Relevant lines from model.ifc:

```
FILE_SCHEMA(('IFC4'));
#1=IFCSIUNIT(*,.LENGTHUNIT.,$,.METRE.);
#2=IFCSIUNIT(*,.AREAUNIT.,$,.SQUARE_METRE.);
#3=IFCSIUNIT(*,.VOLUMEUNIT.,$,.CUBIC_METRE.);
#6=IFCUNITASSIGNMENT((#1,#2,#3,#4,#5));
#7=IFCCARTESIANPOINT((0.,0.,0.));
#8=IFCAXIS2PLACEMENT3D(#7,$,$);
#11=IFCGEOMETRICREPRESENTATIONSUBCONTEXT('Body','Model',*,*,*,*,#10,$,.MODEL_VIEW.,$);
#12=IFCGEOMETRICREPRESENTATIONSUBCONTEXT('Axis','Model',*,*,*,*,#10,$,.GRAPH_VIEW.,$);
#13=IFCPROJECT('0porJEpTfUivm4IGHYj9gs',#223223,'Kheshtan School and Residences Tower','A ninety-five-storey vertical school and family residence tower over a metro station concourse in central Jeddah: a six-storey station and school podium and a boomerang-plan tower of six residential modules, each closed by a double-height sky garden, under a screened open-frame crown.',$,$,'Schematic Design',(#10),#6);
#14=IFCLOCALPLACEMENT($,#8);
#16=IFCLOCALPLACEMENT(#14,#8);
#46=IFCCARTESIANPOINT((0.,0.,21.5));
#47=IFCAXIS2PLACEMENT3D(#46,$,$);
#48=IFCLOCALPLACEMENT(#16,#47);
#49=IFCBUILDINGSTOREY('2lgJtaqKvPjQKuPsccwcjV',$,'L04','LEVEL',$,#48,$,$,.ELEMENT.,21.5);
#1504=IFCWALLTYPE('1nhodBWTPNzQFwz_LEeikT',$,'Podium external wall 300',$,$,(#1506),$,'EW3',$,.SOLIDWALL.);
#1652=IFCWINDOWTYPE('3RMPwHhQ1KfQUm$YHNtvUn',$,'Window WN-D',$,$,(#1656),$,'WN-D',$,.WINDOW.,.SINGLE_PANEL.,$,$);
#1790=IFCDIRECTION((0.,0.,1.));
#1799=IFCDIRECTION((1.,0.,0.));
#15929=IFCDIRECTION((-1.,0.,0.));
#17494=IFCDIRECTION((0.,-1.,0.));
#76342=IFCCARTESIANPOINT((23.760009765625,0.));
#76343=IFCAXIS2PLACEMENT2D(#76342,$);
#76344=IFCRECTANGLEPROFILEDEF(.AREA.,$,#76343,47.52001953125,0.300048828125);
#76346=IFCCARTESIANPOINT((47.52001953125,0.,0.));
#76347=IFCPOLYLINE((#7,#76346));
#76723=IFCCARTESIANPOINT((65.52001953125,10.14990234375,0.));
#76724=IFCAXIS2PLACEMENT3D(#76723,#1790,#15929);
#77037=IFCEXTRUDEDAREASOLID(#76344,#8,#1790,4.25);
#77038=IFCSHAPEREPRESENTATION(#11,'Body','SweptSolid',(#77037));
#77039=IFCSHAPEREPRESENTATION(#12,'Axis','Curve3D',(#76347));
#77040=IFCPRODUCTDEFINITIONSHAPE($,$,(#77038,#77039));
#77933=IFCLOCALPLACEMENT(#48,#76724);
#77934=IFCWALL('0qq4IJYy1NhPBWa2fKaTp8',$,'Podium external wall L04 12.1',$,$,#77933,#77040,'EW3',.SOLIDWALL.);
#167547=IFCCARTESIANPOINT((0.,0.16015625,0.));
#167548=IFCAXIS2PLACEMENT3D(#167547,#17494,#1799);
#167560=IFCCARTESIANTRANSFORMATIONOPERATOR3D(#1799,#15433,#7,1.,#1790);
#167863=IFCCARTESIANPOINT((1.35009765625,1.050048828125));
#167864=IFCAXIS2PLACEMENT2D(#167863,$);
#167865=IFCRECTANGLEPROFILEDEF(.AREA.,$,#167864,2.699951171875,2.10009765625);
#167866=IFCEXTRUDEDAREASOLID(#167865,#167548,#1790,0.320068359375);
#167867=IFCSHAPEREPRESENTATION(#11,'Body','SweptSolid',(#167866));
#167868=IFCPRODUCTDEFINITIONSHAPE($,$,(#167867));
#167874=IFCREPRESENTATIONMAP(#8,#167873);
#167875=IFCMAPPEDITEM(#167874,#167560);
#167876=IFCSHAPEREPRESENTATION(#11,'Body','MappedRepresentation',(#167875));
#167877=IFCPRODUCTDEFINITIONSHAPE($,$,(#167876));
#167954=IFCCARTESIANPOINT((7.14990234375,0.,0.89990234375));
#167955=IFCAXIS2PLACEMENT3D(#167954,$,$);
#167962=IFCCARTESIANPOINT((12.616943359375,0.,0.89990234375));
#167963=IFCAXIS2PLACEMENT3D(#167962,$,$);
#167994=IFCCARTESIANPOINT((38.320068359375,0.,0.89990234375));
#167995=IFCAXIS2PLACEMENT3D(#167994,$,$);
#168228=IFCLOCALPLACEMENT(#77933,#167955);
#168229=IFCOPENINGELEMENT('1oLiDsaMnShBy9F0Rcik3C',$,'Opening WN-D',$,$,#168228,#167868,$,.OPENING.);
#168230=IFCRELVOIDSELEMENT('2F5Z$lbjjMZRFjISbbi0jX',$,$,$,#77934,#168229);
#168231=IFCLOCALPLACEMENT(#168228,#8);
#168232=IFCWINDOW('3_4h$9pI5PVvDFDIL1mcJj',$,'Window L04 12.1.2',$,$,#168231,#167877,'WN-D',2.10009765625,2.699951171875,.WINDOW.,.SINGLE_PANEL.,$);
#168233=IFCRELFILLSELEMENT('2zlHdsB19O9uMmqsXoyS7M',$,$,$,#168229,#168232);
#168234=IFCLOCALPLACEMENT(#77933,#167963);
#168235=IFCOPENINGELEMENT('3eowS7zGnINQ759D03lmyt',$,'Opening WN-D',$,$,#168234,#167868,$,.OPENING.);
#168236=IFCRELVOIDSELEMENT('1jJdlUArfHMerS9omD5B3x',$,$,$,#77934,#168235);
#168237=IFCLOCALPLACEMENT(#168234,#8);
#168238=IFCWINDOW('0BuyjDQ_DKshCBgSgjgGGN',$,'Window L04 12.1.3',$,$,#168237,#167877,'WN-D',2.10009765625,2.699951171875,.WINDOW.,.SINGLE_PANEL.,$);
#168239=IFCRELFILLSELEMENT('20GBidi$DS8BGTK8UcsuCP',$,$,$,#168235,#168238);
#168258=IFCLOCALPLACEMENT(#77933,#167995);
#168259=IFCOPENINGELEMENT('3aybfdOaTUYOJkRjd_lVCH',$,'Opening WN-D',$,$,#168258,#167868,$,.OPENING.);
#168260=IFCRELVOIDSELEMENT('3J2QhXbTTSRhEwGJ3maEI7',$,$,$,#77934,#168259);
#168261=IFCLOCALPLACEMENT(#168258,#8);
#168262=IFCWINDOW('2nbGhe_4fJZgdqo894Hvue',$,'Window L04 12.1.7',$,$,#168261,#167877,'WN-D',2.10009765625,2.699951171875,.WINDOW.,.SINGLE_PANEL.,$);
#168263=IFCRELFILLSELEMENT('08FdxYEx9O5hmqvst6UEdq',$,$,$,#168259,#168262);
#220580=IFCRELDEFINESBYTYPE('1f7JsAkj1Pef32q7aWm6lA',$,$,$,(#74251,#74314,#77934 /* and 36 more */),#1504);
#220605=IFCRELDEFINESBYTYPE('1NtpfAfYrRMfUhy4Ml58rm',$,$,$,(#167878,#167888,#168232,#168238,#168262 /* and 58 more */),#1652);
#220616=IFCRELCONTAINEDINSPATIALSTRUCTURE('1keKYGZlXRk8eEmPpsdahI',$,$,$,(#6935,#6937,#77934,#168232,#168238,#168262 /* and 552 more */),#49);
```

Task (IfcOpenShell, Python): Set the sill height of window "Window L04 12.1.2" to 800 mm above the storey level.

```python
import numpy as np
import ifcopenshell
import ifcopenshell.api.geometry
import ifcopenshell.geom
import ifcopenshell.util.element
import ifcopenshell.util.placement
import ifcopenshell.util.shape
import ifcopenshell.util.unit

model = ifcopenshell.open("model.ifc")
unit_scale = ifcopenshell.util.unit.calculate_unit_scale(model)

window = model.by_guid("3_4h$9pI5PVvDFDIL1mcJj")
opening = window.FillsVoids[0].RelatingOpeningElement
storey = ifcopenshell.util.element.get_container(window, ifc_class="IfcBuildingStorey")
level = ifcopenshell.util.placement.get_local_placement(storey.ObjectPlacement)[2, 3]

# The opening's origin need not be at the sill, so measure its lowest point.
shape = ifcopenshell.geom.create_shape(ifcopenshell.geom.settings(), opening)
bottom = ifcopenshell.util.shape.get_shape_bottom_elevation(shape, shape.geometry) / unit_scale
dz = level + 0.8 - bottom

shift = np.array([0.0, 0.0, dz])
# The window is placed relative to its opening, so it follows when the opening moves.
matrix = ifcopenshell.util.placement.get_local_placement(opening.ObjectPlacement)
matrix[:3, 3] += shift
ifcopenshell.api.geometry.edit_object_placement(
    model, product=opening, matrix=matrix, is_si=False, should_transform_children=True
)

print(f"moved by {dz * unit_scale:+.3f} m")

model.write("model_rev.ifc")
```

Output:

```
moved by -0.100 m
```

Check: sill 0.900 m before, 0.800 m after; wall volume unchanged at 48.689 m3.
